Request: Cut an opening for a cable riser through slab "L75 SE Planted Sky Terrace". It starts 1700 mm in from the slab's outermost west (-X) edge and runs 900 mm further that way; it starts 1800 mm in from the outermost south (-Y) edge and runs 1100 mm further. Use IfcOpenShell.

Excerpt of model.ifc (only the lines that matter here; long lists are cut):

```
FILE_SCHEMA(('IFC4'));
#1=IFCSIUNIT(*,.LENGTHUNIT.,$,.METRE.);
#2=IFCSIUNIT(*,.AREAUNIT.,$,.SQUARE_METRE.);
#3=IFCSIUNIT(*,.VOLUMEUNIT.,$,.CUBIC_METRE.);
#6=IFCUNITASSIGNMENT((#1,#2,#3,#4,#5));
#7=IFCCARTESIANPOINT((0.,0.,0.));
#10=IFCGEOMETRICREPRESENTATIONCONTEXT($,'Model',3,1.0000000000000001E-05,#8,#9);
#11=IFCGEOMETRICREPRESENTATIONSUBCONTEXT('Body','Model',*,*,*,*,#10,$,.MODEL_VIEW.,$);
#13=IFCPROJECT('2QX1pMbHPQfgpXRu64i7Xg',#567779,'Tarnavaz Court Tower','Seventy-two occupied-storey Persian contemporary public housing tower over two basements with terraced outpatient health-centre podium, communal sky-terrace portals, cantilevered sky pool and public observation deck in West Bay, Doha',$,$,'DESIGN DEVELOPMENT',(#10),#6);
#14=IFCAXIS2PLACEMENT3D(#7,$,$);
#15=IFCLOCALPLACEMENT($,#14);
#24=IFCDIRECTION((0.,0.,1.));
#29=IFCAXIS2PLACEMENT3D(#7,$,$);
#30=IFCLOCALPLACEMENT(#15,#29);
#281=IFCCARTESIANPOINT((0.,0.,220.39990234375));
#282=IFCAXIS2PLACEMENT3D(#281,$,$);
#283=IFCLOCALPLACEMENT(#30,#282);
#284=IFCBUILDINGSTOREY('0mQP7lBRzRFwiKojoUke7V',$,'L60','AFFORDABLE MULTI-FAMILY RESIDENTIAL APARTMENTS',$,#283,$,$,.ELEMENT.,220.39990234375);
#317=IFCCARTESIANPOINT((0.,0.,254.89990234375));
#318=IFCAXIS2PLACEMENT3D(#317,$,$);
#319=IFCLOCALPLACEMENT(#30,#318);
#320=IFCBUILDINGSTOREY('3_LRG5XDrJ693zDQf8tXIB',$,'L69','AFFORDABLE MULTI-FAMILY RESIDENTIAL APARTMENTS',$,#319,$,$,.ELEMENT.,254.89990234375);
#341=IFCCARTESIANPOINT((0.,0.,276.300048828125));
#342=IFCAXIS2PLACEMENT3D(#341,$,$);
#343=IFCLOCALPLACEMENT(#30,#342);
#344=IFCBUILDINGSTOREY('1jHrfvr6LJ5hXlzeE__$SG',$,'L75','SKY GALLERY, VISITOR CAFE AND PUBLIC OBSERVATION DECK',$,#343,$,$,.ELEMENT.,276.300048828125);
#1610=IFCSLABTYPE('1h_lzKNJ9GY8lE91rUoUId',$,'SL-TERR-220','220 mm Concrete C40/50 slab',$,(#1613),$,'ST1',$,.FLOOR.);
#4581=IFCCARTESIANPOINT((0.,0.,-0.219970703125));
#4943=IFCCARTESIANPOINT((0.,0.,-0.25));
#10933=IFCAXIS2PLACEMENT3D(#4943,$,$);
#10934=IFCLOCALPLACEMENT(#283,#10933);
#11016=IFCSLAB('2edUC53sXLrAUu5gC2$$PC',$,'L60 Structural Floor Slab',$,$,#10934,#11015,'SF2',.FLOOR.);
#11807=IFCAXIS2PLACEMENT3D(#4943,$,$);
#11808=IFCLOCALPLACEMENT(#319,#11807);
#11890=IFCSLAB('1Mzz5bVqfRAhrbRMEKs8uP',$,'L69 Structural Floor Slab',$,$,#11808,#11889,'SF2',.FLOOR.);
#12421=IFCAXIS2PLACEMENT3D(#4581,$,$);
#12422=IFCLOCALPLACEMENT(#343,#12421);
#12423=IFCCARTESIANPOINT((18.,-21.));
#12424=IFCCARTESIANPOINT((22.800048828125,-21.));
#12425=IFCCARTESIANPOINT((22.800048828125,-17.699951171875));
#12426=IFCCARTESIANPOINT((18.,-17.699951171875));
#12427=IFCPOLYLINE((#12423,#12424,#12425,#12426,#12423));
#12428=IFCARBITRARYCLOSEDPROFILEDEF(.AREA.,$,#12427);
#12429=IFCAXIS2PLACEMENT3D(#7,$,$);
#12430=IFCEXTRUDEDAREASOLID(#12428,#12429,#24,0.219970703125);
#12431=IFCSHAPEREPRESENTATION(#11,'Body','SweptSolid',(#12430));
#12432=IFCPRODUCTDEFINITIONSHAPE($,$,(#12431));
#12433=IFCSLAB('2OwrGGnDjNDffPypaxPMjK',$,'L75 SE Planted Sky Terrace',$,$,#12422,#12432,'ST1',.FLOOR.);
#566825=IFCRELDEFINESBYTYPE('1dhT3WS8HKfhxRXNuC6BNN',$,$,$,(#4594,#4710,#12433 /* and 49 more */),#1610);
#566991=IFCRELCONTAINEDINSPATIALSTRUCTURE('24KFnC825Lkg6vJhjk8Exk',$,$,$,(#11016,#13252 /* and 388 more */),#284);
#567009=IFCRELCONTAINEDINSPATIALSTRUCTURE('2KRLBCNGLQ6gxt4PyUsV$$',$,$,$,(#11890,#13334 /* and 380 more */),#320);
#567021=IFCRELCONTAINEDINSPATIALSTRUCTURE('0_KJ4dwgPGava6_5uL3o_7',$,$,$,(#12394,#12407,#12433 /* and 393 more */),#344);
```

```python
import numpy as np
import ifcopenshell
import ifcopenshell.api.feature
import ifcopenshell.api.geometry
import ifcopenshell.api.root
import ifcopenshell.geom
import ifcopenshell.util.placement
import ifcopenshell.util.representation
import ifcopenshell.util.shape
import ifcopenshell.util.unit

model = ifcopenshell.open("model.ifc")
unit_scale = ifcopenshell.util.unit.calculate_unit_scale(model)
settings = ifcopenshell.geom.settings()


def volume(element):
    """Net volume in cubic metres, openings subtracted."""
    shape = ifcopenshell.geom.create_shape(settings, element)
    return ifcopenshell.util.shape.get_volume(shape.geometry)


slab = model.by_id(12433)
before = volume(slab)

# Extent in the slab's own axes, in metres. The edges named are its -X and -Y sides.
slab_shape = ifcopenshell.geom.create_shape(settings, slab)
vertices = ifcopenshell.util.shape.get_vertices(slab_shape.geometry)
x_min, y_min, bottom = vertices.min(axis=0)
top = vertices[:, 2].max()

opening = ifcopenshell.api.root.create_entity(model, ifc_class="IfcOpeningElement", name="Cable riser opening", predefined_type="OPENING")
context = ifcopenshell.util.representation.get_context(model, "Model", "Body", "MODEL_VIEW")
width, depth = 0.9, 1.1
outline = [(0.0, 0.0), (width, 0.0), (width, depth), (0.0, depth), (0.0, 0.0)]
# Overshoot both faces by 50 mm so the cut is clean.
shape = ifcopenshell.api.geometry.add_slab_representation(
    model, context=context, depth=top - bottom + 0.1, polyline=outline
)
ifcopenshell.api.geometry.assign_representation(model, product=opening, representation=shape)

matrix = ifcopenshell.util.placement.get_local_placement(slab.ObjectPlacement)
matrix[:, 3] = matrix @ np.append(np.array([x_min + 1.7, y_min + 1.8, bottom - 0.05]) / unit_scale, 1.0)
ifcopenshell.api.geometry.edit_object_placement(model, product=opening, matrix=matrix, is_si=False)
ifcopenshell.api.feature.add_feature(model, feature=opening, element=slab)

after = volume(slab)

print(f"slab volume {before:.3f} -> {after:.3f} m3")

model.write("model_rev.ifc")
```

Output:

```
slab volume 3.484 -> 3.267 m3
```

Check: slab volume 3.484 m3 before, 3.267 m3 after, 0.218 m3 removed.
